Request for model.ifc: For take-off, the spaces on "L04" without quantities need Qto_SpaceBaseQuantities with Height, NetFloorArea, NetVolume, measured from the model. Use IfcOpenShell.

First a look at what the model holds.

```python
import ifcopenshell
import ifcopenshell.util.element
import ifcopenshell.util.unit

model = ifcopenshell.open("model.ifc")
print(model.schema)
for unit_type in ("LENGTHUNIT", "AREAUNIT", "VOLUMEUNIT"):
    print(unit_type, ifcopenshell.util.unit.calculate_unit_scale(model, unit_type))
storey = next(s for s in model.by_type("IfcBuildingStorey") if s.Name == "L04")
spaces = [e for e in ifcopenshell.util.element.get_decomposition(storey) if e.is_a("IfcSpace")]
for e in sorted(spaces, key=lambda e: e.id()):
    print(e.id(), e.is_a(), e.Name, list(ifcopenshell.util.element.get_psets(e, qtos_only=True)), sep=" | ")
```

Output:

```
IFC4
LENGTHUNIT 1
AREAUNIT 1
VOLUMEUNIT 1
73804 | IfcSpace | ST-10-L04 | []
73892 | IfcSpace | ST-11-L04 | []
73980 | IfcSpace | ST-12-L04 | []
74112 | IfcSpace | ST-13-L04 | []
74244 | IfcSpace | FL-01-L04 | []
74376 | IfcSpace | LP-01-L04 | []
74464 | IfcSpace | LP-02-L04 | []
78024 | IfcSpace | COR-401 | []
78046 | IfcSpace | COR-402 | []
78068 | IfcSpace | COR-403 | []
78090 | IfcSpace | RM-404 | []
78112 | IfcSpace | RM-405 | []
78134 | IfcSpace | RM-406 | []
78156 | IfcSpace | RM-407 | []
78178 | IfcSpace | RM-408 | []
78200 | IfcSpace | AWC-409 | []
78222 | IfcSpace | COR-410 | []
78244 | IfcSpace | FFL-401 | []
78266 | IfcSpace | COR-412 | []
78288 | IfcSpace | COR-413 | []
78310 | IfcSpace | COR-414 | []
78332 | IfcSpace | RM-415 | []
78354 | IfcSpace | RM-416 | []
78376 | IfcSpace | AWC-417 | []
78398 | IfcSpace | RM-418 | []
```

```python
import ifcopenshell
import ifcopenshell.api.pset
import ifcopenshell.geom
import ifcopenshell.util.element
import ifcopenshell.util.shape
import ifcopenshell.util.unit

model = ifcopenshell.open("model.ifc")
unit_scale = ifcopenshell.util.unit.calculate_unit_scale(model)
area_scale = ifcopenshell.util.unit.calculate_unit_scale(model, "AREAUNIT")
volume_scale = ifcopenshell.util.unit.calculate_unit_scale(model, "VOLUMEUNIT")
settings = ifcopenshell.geom.settings()

storey = next(s for s in model.by_type("IfcBuildingStorey") if s.Name == "L04")
spaces = [e for e in ifcopenshell.util.element.get_decomposition(storey) if e.is_a("IfcSpace")]

for e in sorted(spaces, key=lambda e: e.id()):
    if ifcopenshell.util.element.get_psets(e, qtos_only=True, should_inherit=False):
        continue
    # Geometry comes back in metres, in the element's own axes.
    shape = ifcopenshell.geom.create_shape(settings, e)
    values = {
        "Height": ifcopenshell.util.shape.get_z(shape.geometry) / unit_scale,
        "NetFloorArea": ifcopenshell.util.shape.get_footprint_area(shape.geometry) / area_scale,
        "NetVolume": ifcopenshell.util.shape.get_volume(shape.geometry) / volume_scale,
    }
    qto = ifcopenshell.api.pset.add_qto(model, product=e, name="Qto_SpaceBaseQuantities")
    ifcopenshell.api.pset.edit_qto(model, qto=qto, properties=values)
    print(e.id(), {k: round(v, 3) for k, v in values.items()})

model.write("model-out.ifc")
```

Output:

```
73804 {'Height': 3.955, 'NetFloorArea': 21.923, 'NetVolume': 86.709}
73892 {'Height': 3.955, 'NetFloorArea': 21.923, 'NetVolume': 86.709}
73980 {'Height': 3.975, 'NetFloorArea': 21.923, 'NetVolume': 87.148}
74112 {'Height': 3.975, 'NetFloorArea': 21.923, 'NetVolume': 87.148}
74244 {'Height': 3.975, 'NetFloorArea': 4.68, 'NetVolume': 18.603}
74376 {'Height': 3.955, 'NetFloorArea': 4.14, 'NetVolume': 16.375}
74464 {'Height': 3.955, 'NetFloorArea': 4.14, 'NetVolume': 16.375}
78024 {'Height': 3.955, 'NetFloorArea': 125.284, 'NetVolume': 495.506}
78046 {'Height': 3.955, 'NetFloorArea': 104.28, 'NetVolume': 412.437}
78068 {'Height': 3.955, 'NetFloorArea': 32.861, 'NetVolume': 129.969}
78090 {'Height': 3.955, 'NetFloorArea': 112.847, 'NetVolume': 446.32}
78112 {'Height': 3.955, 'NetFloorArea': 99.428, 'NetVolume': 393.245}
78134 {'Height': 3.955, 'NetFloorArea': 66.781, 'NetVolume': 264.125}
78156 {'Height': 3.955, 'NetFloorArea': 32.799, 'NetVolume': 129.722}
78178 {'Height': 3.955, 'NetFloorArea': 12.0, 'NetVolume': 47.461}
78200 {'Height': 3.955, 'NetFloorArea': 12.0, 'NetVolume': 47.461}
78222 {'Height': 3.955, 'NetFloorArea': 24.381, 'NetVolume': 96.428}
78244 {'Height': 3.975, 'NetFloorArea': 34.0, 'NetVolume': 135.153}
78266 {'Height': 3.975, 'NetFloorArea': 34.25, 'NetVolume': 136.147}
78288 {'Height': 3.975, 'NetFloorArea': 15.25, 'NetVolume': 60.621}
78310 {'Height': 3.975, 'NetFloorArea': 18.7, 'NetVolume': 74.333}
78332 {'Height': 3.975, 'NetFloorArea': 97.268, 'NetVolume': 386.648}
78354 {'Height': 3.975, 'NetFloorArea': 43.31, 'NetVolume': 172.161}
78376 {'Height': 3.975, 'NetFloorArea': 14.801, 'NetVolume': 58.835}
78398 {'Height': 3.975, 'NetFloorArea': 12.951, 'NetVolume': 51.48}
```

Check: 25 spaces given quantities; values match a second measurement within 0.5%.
